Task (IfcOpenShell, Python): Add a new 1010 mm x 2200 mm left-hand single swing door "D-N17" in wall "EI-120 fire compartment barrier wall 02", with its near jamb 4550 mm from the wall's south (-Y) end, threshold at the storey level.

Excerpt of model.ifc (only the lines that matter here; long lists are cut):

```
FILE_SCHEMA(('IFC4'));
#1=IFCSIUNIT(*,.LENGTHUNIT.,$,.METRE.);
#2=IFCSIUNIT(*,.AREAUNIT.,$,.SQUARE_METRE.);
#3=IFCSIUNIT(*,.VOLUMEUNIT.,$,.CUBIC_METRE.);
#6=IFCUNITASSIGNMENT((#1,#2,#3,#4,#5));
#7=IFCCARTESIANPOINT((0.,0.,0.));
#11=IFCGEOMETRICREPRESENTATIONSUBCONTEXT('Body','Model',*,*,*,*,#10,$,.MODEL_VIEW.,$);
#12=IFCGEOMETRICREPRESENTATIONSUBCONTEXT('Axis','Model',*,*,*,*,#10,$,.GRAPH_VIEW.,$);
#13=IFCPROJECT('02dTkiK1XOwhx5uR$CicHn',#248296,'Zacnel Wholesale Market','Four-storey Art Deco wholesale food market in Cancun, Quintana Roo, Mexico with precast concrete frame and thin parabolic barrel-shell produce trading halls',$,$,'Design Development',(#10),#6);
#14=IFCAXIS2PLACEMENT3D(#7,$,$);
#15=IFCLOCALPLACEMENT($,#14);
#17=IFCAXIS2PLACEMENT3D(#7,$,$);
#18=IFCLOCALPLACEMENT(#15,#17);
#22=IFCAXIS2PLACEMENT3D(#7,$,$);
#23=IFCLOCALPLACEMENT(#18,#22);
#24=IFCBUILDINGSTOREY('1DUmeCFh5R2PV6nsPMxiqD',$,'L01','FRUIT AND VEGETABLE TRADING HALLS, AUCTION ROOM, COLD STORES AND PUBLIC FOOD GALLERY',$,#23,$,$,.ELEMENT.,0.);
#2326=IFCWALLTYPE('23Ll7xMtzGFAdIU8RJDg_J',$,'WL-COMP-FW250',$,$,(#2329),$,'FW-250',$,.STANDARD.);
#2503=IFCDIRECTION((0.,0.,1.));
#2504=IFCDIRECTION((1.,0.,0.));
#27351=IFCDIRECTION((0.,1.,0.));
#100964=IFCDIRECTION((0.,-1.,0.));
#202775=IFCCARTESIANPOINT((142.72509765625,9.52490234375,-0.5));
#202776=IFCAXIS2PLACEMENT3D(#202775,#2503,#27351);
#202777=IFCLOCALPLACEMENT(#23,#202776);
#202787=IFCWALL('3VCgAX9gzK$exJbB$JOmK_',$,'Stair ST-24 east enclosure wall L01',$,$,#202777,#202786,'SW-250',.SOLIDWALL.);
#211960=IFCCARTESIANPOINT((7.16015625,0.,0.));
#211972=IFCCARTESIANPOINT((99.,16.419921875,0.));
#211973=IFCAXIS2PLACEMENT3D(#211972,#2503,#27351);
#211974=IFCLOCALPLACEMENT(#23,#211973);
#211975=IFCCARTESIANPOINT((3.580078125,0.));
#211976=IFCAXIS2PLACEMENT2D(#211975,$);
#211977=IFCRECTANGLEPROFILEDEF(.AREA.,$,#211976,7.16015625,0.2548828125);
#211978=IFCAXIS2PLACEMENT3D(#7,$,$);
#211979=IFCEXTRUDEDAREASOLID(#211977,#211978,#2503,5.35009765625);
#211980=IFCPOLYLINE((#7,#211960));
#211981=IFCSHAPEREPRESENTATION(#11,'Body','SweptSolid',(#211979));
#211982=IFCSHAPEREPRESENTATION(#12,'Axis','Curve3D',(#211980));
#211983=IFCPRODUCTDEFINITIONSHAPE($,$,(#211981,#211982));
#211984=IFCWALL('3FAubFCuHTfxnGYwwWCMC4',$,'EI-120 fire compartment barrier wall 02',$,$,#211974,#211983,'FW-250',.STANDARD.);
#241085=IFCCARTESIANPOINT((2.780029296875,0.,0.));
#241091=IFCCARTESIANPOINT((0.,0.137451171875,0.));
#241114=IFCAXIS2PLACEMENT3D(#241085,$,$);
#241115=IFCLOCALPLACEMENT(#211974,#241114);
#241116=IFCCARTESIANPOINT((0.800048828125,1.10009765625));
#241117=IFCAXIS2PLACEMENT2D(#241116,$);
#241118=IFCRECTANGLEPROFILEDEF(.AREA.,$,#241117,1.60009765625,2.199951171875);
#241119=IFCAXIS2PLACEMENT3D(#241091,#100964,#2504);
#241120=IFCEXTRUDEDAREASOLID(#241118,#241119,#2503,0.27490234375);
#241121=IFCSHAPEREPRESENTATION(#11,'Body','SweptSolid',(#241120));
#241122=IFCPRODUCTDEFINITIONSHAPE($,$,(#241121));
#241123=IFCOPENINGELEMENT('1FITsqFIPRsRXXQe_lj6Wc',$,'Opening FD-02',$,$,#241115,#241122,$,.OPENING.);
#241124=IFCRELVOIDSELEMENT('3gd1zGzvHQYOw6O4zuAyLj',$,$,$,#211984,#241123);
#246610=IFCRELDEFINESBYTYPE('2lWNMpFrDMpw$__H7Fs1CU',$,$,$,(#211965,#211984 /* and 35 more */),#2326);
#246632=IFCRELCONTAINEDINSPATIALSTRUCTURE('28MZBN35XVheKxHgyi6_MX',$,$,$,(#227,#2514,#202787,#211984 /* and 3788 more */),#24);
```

```python
import numpy as np
import ifcopenshell
import ifcopenshell.api.feature
import ifcopenshell.api.geometry
import ifcopenshell.api.root
import ifcopenshell.api.spatial
import ifcopenshell.geom
import ifcopenshell.util.element
import ifcopenshell.util.placement
import ifcopenshell.util.representation
import ifcopenshell.util.shape
import ifcopenshell.util.unit

model = ifcopenshell.open("model.ifc")
unit_scale = ifcopenshell.util.unit.calculate_unit_scale(model)
settings = ifcopenshell.geom.settings()


def volume(element):
    """Net volume in cubic metres, openings subtracted."""
    shape = ifcopenshell.geom.create_shape(settings, element)
    return ifcopenshell.util.shape.get_volume(shape.geometry)


wall = model.by_guid("3FAubFCuHTfxnGYwwWCMC4")
storey = ifcopenshell.util.element.get_container(wall, ifc_class="IfcBuildingStorey")
context = ifcopenshell.util.representation.get_context(model, "Model", "Body", "MODEL_VIEW")
before = volume(wall)

width, height, from_end, sill = 1.01, 2.2, 4.55, 0.0  # metres

# The wall runs along its own X axis, and the end named is its -X end.
wall_shape = ifcopenshell.geom.create_shape(settings, wall)
x, y, z = ifcopenshell.util.shape.get_vertices(wall_shape.geometry).T
start = x.min() + from_end
face, thickness = float(y.min()), float(y.max() - y.min())
wall_matrix = ifcopenshell.util.placement.get_local_placement(wall.ObjectPlacement)
level = ifcopenshell.util.placement.get_local_placement(storey.ObjectPlacement)[2, 3]


def in_wall(x, y):
    """Placement at x, y metres in the wall's axes, at sill height."""
    matrix = wall_matrix.copy()
    matrix[:, 3] = wall_matrix @ np.array([x / unit_scale, y / unit_scale, 0.0, 1.0])
    matrix[2, 3] = level + sill / unit_scale
    return matrix


# Opening: a box that overshoots both wall faces by 50 mm.
opening = ifcopenshell.api.root.create_entity(model, ifc_class="IfcOpeningElement", predefined_type="OPENING")
box = ifcopenshell.api.geometry.add_wall_representation(
    model, context=context, length=width, height=height, thickness=thickness + 0.1
)
ifcopenshell.api.geometry.assign_representation(model, product=opening, representation=box)
ifcopenshell.api.geometry.edit_object_placement(model, product=opening, matrix=in_wall(start, face - 0.05), is_si=False)
ifcopenshell.api.feature.add_feature(model, feature=opening, element=wall)

door = ifcopenshell.api.root.create_entity(model, ifc_class="IfcDoor", name="D-N17", predefined_type="DOOR")
door.OverallWidth, door.OverallHeight = width / unit_scale, height / unit_scale
door.OperationType = "SINGLE_SWING_LEFT"
body = ifcopenshell.api.geometry.add_door_representation(
    model,
    context=context,
    overall_width=door.OverallWidth,
    overall_height=door.OverallHeight,
    operation_type="SINGLE_SWING_LEFT",
    lining_properties={"LiningDepth": thickness / unit_scale, "ThresholdDepth": thickness / unit_scale},
)
ifcopenshell.api.geometry.assign_representation(model, product=door, representation=body)
ifcopenshell.api.spatial.assign_container(model, products=[door], relating_structure=storey)
ifcopenshell.api.feature.add_filling(model, opening=opening, element=door)

# The lining spans the wall, so the door starts at the wall face.
ifcopenshell.api.geometry.edit_object_placement(model, product=door, matrix=in_wall(start, face), is_si=False)

after = volume(wall)

print(f"wall volume {before:.3f} -> {after:.3f} m3")

model.write("model-out.ifc")
```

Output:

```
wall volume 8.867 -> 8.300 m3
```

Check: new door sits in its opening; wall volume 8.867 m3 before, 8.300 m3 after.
